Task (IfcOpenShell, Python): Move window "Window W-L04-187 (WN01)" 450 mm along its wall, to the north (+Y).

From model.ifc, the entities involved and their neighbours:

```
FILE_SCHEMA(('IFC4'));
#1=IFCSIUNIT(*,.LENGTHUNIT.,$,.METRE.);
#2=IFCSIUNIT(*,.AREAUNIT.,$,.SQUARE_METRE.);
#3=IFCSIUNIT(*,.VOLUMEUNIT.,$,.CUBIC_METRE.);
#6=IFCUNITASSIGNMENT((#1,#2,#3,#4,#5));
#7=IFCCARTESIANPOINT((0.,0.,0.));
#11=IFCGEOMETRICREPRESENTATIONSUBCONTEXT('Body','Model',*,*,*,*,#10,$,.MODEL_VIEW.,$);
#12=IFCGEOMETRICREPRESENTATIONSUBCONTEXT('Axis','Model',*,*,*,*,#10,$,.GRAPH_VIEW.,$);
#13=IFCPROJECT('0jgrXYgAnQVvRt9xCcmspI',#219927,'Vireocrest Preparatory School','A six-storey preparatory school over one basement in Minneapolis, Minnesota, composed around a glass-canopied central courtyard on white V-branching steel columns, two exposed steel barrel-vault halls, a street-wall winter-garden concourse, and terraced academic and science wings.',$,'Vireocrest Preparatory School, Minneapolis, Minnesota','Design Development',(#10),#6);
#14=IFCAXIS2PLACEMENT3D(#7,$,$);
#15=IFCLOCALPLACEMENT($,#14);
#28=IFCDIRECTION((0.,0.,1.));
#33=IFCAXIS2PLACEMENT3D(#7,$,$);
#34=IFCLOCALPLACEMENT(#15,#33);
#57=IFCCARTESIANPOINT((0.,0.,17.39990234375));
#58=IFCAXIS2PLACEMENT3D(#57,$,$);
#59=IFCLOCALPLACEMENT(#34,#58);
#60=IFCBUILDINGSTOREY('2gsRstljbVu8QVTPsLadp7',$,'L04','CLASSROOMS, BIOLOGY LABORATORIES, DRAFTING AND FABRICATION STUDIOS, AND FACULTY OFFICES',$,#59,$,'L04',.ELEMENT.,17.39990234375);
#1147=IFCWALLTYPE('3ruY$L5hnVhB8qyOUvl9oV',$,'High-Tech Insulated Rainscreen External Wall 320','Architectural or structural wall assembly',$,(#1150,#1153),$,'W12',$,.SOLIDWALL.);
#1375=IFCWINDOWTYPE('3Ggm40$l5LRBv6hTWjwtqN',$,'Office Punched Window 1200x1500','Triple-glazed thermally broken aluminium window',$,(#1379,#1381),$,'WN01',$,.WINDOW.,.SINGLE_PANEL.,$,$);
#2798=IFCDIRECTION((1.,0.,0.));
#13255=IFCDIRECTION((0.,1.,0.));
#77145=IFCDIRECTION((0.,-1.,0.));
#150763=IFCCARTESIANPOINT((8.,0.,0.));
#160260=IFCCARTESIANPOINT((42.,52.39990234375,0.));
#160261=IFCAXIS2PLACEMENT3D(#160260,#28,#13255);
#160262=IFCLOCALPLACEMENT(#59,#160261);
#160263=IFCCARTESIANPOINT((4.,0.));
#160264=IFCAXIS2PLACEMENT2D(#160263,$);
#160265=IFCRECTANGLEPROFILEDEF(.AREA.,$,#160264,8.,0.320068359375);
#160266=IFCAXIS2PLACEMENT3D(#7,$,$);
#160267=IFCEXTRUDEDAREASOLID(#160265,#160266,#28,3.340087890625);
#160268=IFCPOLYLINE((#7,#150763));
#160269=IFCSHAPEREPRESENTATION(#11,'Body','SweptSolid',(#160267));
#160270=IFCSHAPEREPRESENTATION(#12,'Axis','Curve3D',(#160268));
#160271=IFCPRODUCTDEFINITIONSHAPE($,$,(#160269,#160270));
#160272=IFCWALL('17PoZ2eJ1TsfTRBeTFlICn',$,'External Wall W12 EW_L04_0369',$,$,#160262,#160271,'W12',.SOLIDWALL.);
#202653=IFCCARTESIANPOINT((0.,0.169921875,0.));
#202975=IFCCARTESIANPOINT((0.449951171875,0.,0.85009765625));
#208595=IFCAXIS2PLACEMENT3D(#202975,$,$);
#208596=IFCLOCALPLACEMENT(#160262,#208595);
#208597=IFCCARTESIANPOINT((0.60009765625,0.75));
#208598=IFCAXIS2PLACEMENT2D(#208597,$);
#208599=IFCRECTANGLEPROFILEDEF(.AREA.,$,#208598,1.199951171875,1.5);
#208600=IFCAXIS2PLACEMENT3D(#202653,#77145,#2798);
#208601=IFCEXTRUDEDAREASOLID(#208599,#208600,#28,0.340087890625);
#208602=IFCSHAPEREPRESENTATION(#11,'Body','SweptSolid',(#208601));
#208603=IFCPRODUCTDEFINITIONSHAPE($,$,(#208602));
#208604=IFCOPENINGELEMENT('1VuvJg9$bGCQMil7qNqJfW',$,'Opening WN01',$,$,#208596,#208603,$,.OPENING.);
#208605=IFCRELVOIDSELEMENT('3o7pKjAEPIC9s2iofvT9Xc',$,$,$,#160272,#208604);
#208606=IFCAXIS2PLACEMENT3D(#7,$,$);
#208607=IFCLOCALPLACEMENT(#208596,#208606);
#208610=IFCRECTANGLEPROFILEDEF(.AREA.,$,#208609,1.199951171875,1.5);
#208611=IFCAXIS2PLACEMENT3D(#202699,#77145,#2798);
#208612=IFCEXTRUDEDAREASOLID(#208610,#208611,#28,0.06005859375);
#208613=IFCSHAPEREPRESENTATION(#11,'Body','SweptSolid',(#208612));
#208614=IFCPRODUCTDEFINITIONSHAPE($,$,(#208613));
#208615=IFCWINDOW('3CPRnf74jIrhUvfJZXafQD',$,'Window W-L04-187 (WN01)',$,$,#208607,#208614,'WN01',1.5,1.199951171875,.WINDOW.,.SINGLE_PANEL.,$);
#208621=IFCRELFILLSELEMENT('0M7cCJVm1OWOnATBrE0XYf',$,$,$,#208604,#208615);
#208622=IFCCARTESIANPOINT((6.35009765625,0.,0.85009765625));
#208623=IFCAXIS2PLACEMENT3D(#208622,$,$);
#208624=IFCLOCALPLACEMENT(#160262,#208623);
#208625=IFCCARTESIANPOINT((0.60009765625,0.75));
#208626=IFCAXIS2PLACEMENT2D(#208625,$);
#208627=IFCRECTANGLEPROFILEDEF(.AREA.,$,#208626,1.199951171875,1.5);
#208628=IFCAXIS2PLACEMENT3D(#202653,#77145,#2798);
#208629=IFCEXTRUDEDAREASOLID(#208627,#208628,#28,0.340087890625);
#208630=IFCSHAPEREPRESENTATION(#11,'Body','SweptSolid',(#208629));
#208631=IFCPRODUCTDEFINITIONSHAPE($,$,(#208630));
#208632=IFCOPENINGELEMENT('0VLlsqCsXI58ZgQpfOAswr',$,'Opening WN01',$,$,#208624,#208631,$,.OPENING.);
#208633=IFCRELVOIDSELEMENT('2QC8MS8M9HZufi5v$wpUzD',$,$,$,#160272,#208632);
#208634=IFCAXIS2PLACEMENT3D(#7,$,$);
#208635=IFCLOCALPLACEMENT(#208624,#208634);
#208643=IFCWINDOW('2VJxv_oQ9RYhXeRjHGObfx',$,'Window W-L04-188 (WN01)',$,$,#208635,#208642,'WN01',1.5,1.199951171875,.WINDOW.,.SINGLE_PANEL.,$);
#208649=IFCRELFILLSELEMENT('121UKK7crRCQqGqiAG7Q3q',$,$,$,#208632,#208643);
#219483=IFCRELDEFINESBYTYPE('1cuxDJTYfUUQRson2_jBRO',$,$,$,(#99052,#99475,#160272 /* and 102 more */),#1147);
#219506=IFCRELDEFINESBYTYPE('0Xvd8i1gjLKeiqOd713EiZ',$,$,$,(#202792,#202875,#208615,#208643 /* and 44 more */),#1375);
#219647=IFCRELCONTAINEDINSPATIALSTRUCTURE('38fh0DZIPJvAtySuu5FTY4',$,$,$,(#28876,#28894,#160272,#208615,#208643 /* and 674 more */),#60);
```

```python
import ifcopenshell
import ifcopenshell.api.geometry
import ifcopenshell.util.placement
import ifcopenshell.util.unit

model = ifcopenshell.open("model.ifc")
unit_scale = ifcopenshell.util.unit.calculate_unit_scale(model)

window = model.by_guid("3CPRnf74jIrhUvfJZXafQD")
opening = window.FillsVoids[0].RelatingOpeningElement
wall = opening.VoidsElements[0].RelatingBuildingElement

wall_matrix = ifcopenshell.util.placement.get_local_placement(wall.ObjectPlacement)
shift = wall_matrix[:3, 0] * 0.45 / unit_scale
before = ifcopenshell.util.placement.get_local_placement(window.ObjectPlacement)[:3, 3].copy()

# The window is placed relative to its opening, so it follows when the opening moves.
matrix = ifcopenshell.util.placement.get_local_placement(opening.ObjectPlacement)
matrix[:3, 3] += shift
ifcopenshell.api.geometry.edit_object_placement(
    model, product=opening, matrix=matrix, is_si=False, should_transform_children=True
)

after = ifcopenshell.util.placement.get_local_placement(window.ObjectPlacement)[:3, 3]
print("window moved by", (after - before).round(3) + 0.0)

model.write("model_updated.ifc")
```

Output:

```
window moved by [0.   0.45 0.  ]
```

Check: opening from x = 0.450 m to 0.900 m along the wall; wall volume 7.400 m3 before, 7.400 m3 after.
